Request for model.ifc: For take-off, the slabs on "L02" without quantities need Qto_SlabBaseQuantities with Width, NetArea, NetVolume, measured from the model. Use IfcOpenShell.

First a look at what the model holds.

```python
import ifcopenshell
import ifcopenshell.util.element
import ifcopenshell.util.unit

model = ifcopenshell.open("model.ifc")
print(model.schema)
for unit_type in ("LENGTHUNIT", "AREAUNIT", "VOLUMEUNIT"):
    print(unit_type, ifcopenshell.util.unit.calculate_unit_scale(model, unit_type))
storey = next(s for s in model.by_type("IfcBuildingStorey") if s.Name == "L02")
slabs = [e for e in ifcopenshell.util.element.get_decomposition(storey) if e.is_a("IfcSlab")]
for e in sorted(slabs, key=lambda e: e.id()):
    print(e.id(), e.is_a(), e.Name, list(ifcopenshell.util.element.get_psets(e, qtos_only=True)), sep=" | ")
```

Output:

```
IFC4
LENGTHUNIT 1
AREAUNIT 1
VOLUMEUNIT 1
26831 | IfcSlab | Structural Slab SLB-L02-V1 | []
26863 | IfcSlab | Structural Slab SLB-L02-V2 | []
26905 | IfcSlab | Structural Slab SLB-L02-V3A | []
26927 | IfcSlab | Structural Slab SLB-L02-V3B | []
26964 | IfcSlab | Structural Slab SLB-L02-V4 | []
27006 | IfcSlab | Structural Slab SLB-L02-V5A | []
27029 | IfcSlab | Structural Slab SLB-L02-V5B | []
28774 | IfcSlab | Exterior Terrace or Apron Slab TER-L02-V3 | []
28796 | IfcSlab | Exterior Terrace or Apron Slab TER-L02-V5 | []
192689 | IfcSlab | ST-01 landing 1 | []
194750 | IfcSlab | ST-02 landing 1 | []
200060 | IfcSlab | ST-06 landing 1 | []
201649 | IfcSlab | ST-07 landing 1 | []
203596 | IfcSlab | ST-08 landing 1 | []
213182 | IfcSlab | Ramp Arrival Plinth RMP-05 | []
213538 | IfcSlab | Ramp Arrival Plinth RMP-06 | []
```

```python
import ifcopenshell
import ifcopenshell.api.pset
import ifcopenshell.geom
import ifcopenshell.util.element
import ifcopenshell.util.shape
import ifcopenshell.util.unit

model = ifcopenshell.open("model.ifc")
unit_scale = ifcopenshell.util.unit.calculate_unit_scale(model)
area_scale = ifcopenshell.util.unit.calculate_unit_scale(model, "AREAUNIT")
volume_scale = ifcopenshell.util.unit.calculate_unit_scale(model, "VOLUMEUNIT")
settings = ifcopenshell.geom.settings()

storey = next(s for s in model.by_type("IfcBuildingStorey") if s.Name == "L02")
slabs = [e for e in ifcopenshell.util.element.get_decomposition(storey) if e.is_a("IfcSlab")]

for e in sorted(slabs, key=lambda e: e.id()):
    if ifcopenshell.util.element.get_psets(e, qtos_only=True, should_inherit=False):
        continue
    # Geometry comes back in metres, in the element's own axes.
    shape = ifcopenshell.geom.create_shape(settings, e)
    values = {
        "Width": ifcopenshell.util.shape.get_z(shape.geometry) / unit_scale,
        "NetArea": ifcopenshell.util.shape.get_footprint_area(shape.geometry) / area_scale,
        "NetVolume": ifcopenshell.util.shape.get_volume(shape.geometry) / volume_scale,
    }
    qto = ifcopenshell.api.pset.add_qto(model, product=e, name="Qto_SlabBaseQuantities")
    ifcopenshell.api.pset.edit_qto(model, qto=qto, properties=values)
    print(e.id(), {k: round(v, 3) for k, v in values.items()})

model.write("model_updated.ifc")
```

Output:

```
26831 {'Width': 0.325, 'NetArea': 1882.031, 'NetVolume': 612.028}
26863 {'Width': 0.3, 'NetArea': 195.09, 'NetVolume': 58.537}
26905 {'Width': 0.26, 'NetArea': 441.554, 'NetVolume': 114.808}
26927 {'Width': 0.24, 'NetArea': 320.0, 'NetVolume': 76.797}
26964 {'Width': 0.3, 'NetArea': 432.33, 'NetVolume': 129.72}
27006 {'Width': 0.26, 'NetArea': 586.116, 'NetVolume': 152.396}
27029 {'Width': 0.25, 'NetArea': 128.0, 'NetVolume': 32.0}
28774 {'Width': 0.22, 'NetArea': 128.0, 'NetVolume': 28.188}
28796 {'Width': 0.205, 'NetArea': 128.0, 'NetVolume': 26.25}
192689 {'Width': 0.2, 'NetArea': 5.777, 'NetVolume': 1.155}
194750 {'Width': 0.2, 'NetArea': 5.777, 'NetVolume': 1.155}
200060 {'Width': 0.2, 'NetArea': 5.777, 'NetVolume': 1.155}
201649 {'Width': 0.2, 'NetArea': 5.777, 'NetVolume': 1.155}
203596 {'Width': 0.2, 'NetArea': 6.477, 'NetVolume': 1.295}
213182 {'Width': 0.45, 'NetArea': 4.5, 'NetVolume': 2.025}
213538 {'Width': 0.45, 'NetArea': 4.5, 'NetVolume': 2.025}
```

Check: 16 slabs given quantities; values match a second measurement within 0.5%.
